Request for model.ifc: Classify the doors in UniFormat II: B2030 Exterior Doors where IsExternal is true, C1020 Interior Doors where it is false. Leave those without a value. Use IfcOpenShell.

First a look at what the model holds.

```python
import ifcopenshell
import ifcopenshell.util.element

model = ifcopenshell.open("model.ifc")
print(model.schema)
print("classifications:", [c.Name for c in model.by_type("IfcClassification")])
values = [ifcopenshell.util.element.get_pset(e, "Pset_DoorCommon", "IsExternal") for e in model.by_type("IfcDoor")]
for value in (True, False, None):
    print("IsExternal", value, values.count(value))
```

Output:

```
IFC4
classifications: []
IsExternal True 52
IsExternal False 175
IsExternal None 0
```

```python
import ifcopenshell
import ifcopenshell.api.classification
import ifcopenshell.util.element

model = ifcopenshell.open("model.ifc")

system = ifcopenshell.api.classification.add_classification(model, classification="UniFormat II")

doors = model.by_type("IfcDoor")
external = {e: ifcopenshell.util.element.get_pset(e, "Pset_DoorCommon", "IsExternal") for e in doors}
for flag, code, name in ((True, "B2030", "Exterior Doors"), (False, "C1020", "Interior Doors")):
    products = [e for e in doors if external[e] is flag]
    ifcopenshell.api.classification.add_reference(
        model, products=products, classification=system, identification=code, name=name
    )
    print(code, len(products))

model.write("model_edited.ifc")
```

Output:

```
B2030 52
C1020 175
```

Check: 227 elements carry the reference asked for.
